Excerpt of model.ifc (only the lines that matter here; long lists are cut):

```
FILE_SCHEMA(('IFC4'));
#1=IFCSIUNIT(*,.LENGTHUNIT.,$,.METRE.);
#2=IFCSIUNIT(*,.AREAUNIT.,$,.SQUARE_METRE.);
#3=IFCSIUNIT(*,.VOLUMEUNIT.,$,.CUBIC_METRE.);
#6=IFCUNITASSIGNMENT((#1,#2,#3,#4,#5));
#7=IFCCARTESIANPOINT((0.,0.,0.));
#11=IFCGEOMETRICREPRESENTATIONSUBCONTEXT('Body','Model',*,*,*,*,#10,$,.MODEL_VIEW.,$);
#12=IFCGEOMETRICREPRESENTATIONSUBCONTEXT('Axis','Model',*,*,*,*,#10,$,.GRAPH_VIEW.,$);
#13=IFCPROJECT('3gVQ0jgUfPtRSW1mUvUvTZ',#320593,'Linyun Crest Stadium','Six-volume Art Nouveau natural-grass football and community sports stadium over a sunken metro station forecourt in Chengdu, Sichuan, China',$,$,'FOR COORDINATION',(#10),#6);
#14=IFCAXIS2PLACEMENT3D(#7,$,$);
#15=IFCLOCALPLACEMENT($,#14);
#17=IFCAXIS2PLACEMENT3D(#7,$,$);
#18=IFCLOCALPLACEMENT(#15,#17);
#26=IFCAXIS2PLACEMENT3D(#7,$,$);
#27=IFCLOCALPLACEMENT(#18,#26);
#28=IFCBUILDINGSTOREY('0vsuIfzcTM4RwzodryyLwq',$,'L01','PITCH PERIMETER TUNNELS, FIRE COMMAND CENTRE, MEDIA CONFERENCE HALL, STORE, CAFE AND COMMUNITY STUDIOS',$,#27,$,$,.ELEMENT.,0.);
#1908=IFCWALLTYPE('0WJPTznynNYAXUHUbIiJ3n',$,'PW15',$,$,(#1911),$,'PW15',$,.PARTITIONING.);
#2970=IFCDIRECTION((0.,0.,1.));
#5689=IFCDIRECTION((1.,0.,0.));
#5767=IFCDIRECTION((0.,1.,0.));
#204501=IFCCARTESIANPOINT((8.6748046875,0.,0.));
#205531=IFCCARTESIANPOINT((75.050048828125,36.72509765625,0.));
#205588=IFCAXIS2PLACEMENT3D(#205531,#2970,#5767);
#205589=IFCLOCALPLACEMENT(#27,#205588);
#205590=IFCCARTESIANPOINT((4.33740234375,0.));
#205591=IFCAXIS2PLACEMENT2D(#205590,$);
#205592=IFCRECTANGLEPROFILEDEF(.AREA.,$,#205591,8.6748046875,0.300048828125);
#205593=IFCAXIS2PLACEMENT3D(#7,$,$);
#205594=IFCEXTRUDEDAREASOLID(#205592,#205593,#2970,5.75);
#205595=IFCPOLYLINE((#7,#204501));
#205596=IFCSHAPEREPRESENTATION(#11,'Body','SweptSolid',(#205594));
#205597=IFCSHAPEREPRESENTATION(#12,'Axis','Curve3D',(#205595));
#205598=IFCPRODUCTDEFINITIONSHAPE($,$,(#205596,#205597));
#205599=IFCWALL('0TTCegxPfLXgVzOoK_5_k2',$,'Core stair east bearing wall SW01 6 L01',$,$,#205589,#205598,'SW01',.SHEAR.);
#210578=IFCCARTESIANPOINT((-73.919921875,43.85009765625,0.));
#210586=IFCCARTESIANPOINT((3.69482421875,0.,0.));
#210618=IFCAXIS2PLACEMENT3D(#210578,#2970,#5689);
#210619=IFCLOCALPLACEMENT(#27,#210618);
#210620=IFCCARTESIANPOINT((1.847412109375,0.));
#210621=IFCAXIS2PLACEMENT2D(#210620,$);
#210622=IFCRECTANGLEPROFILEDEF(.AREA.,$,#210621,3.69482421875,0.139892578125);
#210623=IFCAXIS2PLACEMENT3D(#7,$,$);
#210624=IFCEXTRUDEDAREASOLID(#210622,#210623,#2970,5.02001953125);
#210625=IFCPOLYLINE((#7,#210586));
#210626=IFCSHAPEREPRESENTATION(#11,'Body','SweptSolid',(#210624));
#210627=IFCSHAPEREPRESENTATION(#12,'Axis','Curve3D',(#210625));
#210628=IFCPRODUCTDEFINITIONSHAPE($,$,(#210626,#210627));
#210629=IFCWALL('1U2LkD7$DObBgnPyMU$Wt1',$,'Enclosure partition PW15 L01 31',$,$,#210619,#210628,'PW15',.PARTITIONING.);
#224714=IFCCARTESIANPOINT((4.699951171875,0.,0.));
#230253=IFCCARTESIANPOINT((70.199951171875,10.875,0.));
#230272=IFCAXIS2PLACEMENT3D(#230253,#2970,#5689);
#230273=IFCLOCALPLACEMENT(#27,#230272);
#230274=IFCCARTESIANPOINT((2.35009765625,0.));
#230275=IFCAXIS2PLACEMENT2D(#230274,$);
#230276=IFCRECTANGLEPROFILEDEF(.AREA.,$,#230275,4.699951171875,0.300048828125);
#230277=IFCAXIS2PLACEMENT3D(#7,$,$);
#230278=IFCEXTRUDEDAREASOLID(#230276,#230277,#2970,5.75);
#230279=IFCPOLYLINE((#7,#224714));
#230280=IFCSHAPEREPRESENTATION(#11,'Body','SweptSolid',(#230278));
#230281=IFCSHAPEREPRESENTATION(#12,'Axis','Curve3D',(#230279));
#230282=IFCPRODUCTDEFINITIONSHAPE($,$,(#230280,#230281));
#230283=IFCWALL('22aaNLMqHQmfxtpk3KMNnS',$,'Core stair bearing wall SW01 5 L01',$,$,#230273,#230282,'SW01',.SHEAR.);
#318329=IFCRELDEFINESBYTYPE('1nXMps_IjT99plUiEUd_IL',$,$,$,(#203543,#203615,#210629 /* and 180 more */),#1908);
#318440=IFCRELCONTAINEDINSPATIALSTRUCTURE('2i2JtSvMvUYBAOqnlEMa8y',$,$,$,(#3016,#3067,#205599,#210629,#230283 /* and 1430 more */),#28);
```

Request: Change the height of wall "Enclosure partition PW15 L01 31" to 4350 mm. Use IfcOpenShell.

```python
import ifcopenshell
import ifcopenshell.geom
import ifcopenshell.util.representation
import ifcopenshell.util.shape
import ifcopenshell.util.unit

model = ifcopenshell.open("model.ifc")
unit_scale = ifcopenshell.util.unit.calculate_unit_scale(model)
settings = ifcopenshell.geom.settings()


def volume(element):
    """Net volume in cubic metres, openings subtracted."""
    shape = ifcopenshell.geom.create_shape(settings, element)
    return ifcopenshell.util.shape.get_volume(shape.geometry)


wall = model.by_id(210629)
before = volume(wall)

body = ifcopenshell.util.representation.get_representation(wall, "Model", "Body")
solid = body.Items[0]
old_height = solid.Depth
solid.Depth = 4.35 / unit_scale
after = volume(wall)

print(f"height {old_height:g} -> {solid.Depth:g}, volume {before:.3f} -> {after:.3f} m3")

model.write("model-out.ifc")
```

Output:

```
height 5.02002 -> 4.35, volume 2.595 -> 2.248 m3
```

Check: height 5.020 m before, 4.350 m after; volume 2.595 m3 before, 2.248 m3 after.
